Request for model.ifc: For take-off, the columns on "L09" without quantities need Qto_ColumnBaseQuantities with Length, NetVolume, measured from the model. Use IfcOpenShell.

First a look at what the model holds.

```python
import ifcopenshell
import ifcopenshell.util.element
import ifcopenshell.util.unit

model = ifcopenshell.open("model.ifc")
print(model.schema)
for unit_type in ("LENGTHUNIT", "AREAUNIT", "VOLUMEUNIT"):
    print(unit_type, ifcopenshell.util.unit.calculate_unit_scale(model, unit_type))
storey = next(s for s in model.by_type("IfcBuildingStorey") if s.Name == "L09")
columns = [e for e in ifcopenshell.util.element.get_decomposition(storey) if e.is_a("IfcColumn")]
for e in sorted(columns, key=lambda e: e.id()):
    print(e.id(), e.is_a(), e.Name, list(ifcopenshell.util.element.get_psets(e, qtos_only=True)), sep=" | ")
```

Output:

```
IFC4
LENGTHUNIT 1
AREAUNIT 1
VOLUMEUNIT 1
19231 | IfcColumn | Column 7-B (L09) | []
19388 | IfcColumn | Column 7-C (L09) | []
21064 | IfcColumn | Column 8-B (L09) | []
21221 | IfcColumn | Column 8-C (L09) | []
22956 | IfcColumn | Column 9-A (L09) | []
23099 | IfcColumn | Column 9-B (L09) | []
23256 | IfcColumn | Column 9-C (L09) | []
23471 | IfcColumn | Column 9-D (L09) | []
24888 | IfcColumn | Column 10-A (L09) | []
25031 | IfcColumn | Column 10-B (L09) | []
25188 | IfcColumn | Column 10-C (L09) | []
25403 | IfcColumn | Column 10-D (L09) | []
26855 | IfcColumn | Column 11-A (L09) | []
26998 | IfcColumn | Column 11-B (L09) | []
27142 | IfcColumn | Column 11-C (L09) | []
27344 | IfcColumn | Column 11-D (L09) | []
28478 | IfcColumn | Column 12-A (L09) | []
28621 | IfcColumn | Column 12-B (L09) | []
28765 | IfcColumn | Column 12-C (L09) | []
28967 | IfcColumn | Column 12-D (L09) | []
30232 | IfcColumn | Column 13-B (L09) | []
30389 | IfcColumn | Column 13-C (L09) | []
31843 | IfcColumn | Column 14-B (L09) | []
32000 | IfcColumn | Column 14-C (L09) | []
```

```python
import ifcopenshell
import ifcopenshell.api.pset
import ifcopenshell.geom
import ifcopenshell.util.element
import ifcopenshell.util.shape
import ifcopenshell.util.unit

model = ifcopenshell.open("model.ifc")
unit_scale = ifcopenshell.util.unit.calculate_unit_scale(model)
volume_scale = ifcopenshell.util.unit.calculate_unit_scale(model, "VOLUMEUNIT")
settings = ifcopenshell.geom.settings()

storey = next(s for s in model.by_type("IfcBuildingStorey") if s.Name == "L09")
columns = [e for e in ifcopenshell.util.element.get_decomposition(storey) if e.is_a("IfcColumn")]

for e in sorted(columns, key=lambda e: e.id()):
    if ifcopenshell.util.element.get_psets(e, qtos_only=True, should_inherit=False):
        continue
    # Geometry comes back in metres, in the element's own axes.
    shape = ifcopenshell.geom.create_shape(settings, e)
    values = {
        "Length": ifcopenshell.util.shape.get_z(shape.geometry) / unit_scale,
        "NetVolume": ifcopenshell.util.shape.get_volume(shape.geometry) / volume_scale,
    }
    qto = ifcopenshell.api.pset.add_qto(model, product=e, name="Qto_ColumnBaseQuantities")
    ifcopenshell.api.pset.edit_qto(model, qto=qto, properties=values)
    print(e.id(), {k: round(v, 3) for k, v in values.items()})

model.write("model_updated.ifc")
```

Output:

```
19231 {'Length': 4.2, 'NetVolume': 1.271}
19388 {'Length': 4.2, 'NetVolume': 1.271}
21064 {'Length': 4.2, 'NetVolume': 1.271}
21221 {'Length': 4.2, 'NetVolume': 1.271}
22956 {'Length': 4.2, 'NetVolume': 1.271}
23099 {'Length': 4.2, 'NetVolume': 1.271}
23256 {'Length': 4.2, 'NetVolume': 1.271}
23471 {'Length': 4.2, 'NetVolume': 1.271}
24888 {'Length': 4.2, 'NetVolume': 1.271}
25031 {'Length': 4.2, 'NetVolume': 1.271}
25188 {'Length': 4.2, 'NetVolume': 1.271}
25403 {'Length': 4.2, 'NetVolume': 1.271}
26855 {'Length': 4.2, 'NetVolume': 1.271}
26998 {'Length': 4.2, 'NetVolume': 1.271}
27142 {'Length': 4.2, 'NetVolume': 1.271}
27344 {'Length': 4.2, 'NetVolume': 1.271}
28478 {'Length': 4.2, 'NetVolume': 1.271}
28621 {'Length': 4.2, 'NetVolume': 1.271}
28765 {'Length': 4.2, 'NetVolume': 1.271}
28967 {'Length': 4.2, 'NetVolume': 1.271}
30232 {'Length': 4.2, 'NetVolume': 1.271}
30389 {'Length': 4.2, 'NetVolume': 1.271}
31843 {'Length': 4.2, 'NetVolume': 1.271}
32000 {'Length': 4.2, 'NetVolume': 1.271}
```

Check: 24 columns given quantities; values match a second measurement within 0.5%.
